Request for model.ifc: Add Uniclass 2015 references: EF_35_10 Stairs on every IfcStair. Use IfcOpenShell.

First a look at what the model holds.

```python
import ifcopenshell

model = ifcopenshell.open("model.ifc")
print(model.schema)
print("classifications:", [c.Name for c in model.by_type("IfcClassification")])
for ifc_class in ("IfcDoor", "IfcRoof", "IfcStair", "IfcWall", "IfcWindow"):
    print(ifc_class, len(model.by_type(ifc_class)))
```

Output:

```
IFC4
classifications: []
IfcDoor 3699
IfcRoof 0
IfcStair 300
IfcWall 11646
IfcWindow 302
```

```python
import ifcopenshell
import ifcopenshell.api.classification

model = ifcopenshell.open("model.ifc")

system = ifcopenshell.api.classification.add_classification(model, classification="Uniclass 2015")

codes = {
    "IfcStair": ("EF_35_10", "Stairs"),
}
for ifc_class, (code, name) in codes.items():
    products = model.by_type(ifc_class)
    ifcopenshell.api.classification.add_reference(
        model, products=products, classification=system, identification=code, name=name
    )
    print(code, len(products))

model.write("model_rev.ifc")
```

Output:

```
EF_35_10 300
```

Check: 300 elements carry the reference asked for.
